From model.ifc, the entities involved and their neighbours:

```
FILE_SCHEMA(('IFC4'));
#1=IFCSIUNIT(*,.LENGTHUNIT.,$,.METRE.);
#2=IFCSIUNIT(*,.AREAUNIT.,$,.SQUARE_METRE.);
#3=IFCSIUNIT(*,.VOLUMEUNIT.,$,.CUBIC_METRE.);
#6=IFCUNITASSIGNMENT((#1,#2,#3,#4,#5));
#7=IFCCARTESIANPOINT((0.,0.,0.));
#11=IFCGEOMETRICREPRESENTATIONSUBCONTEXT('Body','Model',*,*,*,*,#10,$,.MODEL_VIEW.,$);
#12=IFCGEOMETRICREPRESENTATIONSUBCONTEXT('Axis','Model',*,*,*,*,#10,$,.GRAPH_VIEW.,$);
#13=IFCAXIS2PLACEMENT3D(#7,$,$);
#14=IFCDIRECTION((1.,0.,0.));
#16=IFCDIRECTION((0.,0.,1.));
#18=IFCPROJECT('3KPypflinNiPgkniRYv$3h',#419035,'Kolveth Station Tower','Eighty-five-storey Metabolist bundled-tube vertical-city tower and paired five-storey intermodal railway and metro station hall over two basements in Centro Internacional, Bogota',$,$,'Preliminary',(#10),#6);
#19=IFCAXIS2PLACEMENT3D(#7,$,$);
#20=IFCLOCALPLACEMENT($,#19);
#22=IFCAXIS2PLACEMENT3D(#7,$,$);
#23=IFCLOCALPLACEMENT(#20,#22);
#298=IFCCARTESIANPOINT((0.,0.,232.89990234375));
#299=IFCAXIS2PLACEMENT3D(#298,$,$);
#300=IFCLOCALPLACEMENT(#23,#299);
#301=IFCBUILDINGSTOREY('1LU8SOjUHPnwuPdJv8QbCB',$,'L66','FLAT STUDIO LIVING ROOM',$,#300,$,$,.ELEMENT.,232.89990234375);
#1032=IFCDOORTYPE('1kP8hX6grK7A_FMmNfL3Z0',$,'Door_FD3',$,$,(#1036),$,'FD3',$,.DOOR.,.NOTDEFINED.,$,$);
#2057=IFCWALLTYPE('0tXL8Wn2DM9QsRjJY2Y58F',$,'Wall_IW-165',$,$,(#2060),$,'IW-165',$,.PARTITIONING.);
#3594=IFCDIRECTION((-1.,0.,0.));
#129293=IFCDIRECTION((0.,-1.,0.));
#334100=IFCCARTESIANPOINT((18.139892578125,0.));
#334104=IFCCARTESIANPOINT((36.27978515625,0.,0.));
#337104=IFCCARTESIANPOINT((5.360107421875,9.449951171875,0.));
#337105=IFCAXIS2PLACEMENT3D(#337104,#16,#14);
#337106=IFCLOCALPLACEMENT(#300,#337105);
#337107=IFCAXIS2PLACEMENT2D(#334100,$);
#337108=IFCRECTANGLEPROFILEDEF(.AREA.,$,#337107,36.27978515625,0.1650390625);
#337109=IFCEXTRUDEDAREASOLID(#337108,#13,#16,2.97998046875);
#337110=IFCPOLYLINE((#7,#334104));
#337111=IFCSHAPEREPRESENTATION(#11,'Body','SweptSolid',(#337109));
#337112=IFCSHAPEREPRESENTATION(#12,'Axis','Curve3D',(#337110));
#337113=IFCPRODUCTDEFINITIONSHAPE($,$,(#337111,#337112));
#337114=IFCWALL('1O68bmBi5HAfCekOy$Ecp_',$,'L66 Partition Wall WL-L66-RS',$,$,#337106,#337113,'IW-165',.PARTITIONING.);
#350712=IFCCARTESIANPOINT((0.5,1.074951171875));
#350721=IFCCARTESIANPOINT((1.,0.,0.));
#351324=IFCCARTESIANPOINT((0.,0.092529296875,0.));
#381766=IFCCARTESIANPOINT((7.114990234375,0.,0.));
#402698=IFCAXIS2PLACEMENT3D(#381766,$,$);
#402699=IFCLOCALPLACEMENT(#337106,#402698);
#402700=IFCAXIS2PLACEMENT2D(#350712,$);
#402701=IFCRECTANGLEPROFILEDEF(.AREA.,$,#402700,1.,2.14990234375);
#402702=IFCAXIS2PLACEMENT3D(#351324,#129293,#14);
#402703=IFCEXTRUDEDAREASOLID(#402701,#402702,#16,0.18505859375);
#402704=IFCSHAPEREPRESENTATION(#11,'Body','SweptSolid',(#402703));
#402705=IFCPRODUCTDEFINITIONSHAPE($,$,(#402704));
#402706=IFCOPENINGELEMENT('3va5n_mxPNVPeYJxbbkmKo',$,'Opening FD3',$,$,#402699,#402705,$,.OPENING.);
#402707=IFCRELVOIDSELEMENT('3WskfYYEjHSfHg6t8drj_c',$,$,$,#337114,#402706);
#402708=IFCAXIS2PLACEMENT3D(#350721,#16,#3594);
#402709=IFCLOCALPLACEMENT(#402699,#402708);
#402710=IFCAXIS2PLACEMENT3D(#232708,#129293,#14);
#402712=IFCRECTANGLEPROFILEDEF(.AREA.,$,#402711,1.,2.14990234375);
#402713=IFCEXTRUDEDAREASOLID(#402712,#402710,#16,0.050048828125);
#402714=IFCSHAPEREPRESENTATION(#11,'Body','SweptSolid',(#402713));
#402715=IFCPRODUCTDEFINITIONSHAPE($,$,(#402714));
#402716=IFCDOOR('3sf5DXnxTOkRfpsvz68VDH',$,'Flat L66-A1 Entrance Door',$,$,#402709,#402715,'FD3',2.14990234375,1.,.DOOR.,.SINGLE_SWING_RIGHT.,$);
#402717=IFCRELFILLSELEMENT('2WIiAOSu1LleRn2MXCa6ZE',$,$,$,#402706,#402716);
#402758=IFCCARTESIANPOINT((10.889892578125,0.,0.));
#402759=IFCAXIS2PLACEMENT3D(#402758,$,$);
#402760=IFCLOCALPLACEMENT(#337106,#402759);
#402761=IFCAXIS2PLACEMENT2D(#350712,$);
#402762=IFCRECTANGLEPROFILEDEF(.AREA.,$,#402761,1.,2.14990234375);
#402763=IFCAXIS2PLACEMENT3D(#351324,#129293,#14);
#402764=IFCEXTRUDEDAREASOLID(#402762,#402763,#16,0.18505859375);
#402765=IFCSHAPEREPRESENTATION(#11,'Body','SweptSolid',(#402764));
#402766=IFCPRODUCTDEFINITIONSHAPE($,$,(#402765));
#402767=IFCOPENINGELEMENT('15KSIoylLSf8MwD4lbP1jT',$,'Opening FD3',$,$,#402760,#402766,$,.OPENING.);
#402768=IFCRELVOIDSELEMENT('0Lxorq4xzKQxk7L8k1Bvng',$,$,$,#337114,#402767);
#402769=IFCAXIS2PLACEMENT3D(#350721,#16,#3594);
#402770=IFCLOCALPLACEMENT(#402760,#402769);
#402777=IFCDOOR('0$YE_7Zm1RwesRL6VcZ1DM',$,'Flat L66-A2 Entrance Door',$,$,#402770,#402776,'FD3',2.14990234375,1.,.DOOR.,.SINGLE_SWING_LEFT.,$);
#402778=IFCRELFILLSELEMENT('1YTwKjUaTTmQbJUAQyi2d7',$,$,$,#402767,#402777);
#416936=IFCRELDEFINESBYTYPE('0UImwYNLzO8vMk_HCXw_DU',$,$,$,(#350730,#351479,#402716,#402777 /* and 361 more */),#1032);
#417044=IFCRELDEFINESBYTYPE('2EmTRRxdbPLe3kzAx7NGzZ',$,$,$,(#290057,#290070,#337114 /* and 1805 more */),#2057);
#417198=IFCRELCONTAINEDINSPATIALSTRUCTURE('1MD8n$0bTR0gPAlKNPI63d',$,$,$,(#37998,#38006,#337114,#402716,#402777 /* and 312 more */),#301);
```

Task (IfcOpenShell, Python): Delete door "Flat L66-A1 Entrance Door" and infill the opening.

```python
import ifcopenshell
import ifcopenshell.api.feature
import ifcopenshell.api.root
import ifcopenshell.geom
import ifcopenshell.util.shape

model = ifcopenshell.open("model.ifc")
settings = ifcopenshell.geom.settings()


def volume(element):
    """Net volume in cubic metres, openings subtracted."""
    shape = ifcopenshell.geom.create_shape(settings, element)
    return ifcopenshell.util.shape.get_volume(shape.geometry)


door = model.by_guid("3sf5DXnxTOkRfpsvz68VDH")
opening = door.FillsVoids[0].RelatingOpeningElement
wall = opening.VoidsElements[0].RelatingBuildingElement
before = volume(wall)

ifcopenshell.api.root.remove_product(model, product=door)
ifcopenshell.api.feature.remove_feature(model, feature=opening)

after = volume(wall)

print(f"wall volume {before:.3f} -> {after:.3f} m3")

model.write("model_edited.ifc")
```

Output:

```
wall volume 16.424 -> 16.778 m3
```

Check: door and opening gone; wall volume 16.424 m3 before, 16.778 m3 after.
